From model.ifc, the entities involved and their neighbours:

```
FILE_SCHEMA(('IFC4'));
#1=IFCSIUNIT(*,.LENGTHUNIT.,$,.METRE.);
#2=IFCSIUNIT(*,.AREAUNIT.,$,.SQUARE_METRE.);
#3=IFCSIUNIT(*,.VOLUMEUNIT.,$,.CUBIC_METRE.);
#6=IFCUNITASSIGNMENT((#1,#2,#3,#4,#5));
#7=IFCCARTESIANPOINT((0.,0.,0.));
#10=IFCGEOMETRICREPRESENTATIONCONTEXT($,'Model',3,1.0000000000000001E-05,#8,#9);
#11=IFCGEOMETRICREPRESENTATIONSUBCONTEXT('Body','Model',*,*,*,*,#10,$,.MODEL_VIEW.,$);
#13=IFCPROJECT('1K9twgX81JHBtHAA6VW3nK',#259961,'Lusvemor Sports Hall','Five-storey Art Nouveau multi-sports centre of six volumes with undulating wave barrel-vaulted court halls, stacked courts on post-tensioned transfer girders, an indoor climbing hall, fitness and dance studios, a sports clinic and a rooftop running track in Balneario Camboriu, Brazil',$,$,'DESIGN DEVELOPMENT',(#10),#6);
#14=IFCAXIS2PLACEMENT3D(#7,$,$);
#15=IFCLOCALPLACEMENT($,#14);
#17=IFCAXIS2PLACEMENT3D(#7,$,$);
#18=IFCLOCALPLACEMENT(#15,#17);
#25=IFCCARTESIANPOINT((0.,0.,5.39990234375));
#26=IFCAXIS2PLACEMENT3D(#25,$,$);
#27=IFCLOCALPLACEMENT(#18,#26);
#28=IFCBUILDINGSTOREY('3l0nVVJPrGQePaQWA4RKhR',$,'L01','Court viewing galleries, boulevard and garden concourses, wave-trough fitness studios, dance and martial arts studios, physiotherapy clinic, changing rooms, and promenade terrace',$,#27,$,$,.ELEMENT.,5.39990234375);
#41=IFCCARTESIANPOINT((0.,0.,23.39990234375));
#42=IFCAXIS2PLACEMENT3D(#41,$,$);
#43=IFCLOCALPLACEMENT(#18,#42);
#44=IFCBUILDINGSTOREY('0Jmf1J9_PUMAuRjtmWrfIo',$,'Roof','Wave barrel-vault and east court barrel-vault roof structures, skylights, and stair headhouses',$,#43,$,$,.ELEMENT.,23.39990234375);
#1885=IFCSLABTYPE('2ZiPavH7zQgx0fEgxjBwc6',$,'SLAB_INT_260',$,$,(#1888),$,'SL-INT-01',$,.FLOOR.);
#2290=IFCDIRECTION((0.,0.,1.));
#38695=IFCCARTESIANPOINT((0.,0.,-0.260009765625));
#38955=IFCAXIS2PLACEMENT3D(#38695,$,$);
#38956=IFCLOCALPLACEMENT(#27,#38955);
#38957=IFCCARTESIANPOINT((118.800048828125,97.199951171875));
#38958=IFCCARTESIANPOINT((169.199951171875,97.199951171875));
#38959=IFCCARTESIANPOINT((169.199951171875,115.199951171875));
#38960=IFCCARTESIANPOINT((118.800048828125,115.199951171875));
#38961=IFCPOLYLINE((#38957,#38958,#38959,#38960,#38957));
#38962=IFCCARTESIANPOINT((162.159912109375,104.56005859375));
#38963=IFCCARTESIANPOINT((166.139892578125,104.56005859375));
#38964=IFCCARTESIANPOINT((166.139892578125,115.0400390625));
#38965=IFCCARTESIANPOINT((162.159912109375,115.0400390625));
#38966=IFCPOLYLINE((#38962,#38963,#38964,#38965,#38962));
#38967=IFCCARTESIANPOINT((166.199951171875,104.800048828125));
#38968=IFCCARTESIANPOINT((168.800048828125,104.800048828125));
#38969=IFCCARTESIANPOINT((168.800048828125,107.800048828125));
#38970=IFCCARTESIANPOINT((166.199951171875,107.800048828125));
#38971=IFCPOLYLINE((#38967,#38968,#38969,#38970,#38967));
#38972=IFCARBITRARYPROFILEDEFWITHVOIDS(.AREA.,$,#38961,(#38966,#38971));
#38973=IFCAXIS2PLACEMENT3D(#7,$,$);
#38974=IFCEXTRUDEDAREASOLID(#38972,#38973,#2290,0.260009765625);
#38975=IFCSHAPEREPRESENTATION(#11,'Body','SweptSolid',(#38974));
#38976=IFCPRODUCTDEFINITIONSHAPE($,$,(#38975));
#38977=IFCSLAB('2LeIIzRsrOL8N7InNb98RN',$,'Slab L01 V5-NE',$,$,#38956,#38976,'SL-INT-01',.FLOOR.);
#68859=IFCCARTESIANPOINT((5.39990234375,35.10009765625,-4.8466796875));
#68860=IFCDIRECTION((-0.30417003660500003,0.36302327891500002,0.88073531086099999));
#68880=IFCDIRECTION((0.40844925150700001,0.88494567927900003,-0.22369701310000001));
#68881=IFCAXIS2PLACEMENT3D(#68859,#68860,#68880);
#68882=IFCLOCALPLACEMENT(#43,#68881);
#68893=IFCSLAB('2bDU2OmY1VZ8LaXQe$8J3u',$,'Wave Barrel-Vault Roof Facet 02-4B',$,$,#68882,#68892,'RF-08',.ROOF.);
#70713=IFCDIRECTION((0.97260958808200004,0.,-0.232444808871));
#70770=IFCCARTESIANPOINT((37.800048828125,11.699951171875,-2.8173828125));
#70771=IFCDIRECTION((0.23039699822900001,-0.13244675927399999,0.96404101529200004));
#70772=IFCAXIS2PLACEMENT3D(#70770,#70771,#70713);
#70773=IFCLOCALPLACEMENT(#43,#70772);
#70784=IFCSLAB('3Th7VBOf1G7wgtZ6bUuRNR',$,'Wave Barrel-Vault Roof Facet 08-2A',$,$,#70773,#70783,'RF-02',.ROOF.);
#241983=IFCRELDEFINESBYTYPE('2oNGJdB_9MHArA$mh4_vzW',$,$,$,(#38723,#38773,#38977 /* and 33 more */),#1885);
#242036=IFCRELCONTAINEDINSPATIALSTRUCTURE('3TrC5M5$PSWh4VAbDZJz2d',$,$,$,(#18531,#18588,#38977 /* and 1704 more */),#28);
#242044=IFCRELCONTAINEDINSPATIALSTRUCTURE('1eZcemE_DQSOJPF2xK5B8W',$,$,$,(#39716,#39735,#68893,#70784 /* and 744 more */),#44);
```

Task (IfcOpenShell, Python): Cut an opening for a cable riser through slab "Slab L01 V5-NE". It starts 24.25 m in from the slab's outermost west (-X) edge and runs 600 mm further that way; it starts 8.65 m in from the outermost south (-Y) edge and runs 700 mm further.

```python
import numpy as np
import ifcopenshell
import ifcopenshell.api.feature
import ifcopenshell.api.geometry
import ifcopenshell.api.root
import ifcopenshell.geom
import ifcopenshell.util.placement
import ifcopenshell.util.representation
import ifcopenshell.util.shape
import ifcopenshell.util.unit

model = ifcopenshell.open("model.ifc")
unit_scale = ifcopenshell.util.unit.calculate_unit_scale(model)
settings = ifcopenshell.geom.settings()


def volume(element):
    """Net volume in cubic metres, openings subtracted."""
    shape = ifcopenshell.geom.create_shape(settings, element)
    return ifcopenshell.util.shape.get_volume(shape.geometry)


slab = model.by_guid("2LeIIzRsrOL8N7InNb98RN")
before = volume(slab)

# Extent in the slab's own axes, in metres. The edges named are its -X and -Y sides.
slab_shape = ifcopenshell.geom.create_shape(settings, slab)
vertices = ifcopenshell.util.shape.get_vertices(slab_shape.geometry)
x_min, y_min, bottom = vertices.min(axis=0)
top = vertices[:, 2].max()

opening = ifcopenshell.api.root.create_entity(model, ifc_class="IfcOpeningElement", name="Cable riser opening", predefined_type="OPENING")
context = ifcopenshell.util.representation.get_context(model, "Model", "Body", "MODEL_VIEW")
width, depth = 0.6, 0.7
outline = [(0.0, 0.0), (width, 0.0), (width, depth), (0.0, depth), (0.0, 0.0)]
# Overshoot both faces by 50 mm so the cut is clean.
shape = ifcopenshell.api.geometry.add_slab_representation(
    model, context=context, depth=top - bottom + 0.1, polyline=outline
)
ifcopenshell.api.geometry.assign_representation(model, product=opening, representation=shape)

matrix = ifcopenshell.util.placement.get_local_placement(slab.ObjectPlacement)
matrix[:, 3] = matrix @ np.append(np.array([x_min + 24.25, y_min + 8.65, bottom - 0.05]) / unit_scale, 1.0)
ifcopenshell.api.geometry.edit_object_placement(model, product=opening, matrix=matrix, is_si=False)
ifcopenshell.api.feature.add_feature(model, feature=opening, element=slab)

after = volume(slab)

print(f"slab volume {before:.3f} -> {after:.3f} m3")

model.write("model_updated.ifc")
```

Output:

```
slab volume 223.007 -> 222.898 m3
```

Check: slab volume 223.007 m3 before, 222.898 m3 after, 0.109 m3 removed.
